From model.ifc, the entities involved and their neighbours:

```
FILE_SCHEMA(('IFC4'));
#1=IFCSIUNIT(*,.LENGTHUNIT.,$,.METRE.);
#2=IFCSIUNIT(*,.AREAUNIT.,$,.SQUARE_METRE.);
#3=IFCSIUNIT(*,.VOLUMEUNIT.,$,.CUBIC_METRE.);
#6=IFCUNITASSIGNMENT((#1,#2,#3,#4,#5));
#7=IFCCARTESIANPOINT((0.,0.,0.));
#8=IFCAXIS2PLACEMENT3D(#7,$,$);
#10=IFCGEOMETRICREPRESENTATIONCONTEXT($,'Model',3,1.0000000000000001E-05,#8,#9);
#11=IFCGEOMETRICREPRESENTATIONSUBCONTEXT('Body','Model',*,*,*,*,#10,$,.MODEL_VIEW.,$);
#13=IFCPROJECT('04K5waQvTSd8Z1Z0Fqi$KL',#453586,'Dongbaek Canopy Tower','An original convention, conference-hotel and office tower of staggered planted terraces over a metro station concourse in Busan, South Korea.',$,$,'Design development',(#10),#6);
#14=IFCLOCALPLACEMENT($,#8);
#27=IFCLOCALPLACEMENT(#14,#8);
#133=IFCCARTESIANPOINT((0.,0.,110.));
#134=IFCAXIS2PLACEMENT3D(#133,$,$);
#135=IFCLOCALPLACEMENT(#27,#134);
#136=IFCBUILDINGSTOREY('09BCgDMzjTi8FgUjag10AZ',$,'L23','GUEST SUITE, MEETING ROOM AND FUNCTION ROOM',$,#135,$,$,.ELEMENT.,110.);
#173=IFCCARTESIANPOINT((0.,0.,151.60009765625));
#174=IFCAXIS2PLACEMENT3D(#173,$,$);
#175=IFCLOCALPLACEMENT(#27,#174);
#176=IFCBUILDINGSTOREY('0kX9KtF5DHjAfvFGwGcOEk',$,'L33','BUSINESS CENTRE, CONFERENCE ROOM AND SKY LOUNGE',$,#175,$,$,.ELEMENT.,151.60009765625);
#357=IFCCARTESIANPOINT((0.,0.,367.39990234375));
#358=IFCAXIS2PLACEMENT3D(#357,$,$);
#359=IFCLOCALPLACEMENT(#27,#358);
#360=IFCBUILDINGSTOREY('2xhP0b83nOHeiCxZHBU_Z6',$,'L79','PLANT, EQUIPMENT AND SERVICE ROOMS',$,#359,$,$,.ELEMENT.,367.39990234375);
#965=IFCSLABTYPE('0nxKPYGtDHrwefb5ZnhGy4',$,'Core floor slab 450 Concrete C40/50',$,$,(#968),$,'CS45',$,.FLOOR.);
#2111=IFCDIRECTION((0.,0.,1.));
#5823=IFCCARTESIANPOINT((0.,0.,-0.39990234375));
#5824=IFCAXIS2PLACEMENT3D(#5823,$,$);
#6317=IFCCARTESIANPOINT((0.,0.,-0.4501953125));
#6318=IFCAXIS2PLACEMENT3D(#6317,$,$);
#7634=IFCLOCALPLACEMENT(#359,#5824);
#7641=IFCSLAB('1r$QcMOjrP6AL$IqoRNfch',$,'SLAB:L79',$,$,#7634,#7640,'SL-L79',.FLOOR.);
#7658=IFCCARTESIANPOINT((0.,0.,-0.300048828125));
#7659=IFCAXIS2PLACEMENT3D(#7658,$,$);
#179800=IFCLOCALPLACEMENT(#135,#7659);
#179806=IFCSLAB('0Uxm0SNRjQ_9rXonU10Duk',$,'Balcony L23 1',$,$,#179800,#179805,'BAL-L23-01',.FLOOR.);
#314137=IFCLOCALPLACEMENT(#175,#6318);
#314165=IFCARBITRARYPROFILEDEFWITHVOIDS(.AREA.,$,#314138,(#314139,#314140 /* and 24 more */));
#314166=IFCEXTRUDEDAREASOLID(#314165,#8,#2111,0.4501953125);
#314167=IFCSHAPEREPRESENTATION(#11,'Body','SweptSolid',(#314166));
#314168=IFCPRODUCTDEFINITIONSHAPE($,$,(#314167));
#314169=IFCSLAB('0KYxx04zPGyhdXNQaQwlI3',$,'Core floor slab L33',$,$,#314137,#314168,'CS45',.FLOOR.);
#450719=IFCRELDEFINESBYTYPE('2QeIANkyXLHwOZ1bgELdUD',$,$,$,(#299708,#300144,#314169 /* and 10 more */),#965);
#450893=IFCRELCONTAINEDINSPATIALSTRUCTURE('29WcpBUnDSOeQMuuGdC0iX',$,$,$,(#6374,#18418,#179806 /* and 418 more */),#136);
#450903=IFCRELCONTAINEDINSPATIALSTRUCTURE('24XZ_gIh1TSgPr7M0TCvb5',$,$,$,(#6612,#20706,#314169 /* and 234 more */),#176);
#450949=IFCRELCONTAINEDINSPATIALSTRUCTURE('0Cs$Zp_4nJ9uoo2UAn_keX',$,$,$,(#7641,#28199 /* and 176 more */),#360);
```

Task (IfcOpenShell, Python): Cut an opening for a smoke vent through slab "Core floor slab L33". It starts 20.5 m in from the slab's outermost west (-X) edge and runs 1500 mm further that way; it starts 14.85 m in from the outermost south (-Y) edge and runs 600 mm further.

```python
import numpy as np
import ifcopenshell
import ifcopenshell.api.feature
import ifcopenshell.api.geometry
import ifcopenshell.api.root
import ifcopenshell.geom
import ifcopenshell.util.placement
import ifcopenshell.util.representation
import ifcopenshell.util.shape
import ifcopenshell.util.unit

model = ifcopenshell.open("model.ifc")
unit_scale = ifcopenshell.util.unit.calculate_unit_scale(model)
settings = ifcopenshell.geom.settings()


def volume(element):
    """Net volume in cubic metres, openings subtracted."""
    shape = ifcopenshell.geom.create_shape(settings, element)
    return ifcopenshell.util.shape.get_volume(shape.geometry)


slab = model.by_id(314169)
before = volume(slab)

# Extent in the slab's own axes, in metres. The edges named are its -X and -Y sides.
slab_shape = ifcopenshell.geom.create_shape(settings, slab)
vertices = ifcopenshell.util.shape.get_vertices(slab_shape.geometry)
x_min, y_min, bottom = vertices.min(axis=0)
top = vertices[:, 2].max()

opening = ifcopenshell.api.root.create_entity(model, ifc_class="IfcOpeningElement", name="Smoke vent opening", predefined_type="OPENING")
context = ifcopenshell.util.representation.get_context(model, "Model", "Body", "MODEL_VIEW")
width, depth = 1.5, 0.6
outline = [(0.0, 0.0), (width, 0.0), (width, depth), (0.0, depth), (0.0, 0.0)]
# Overshoot both faces by 50 mm so the cut is clean.
shape = ifcopenshell.api.geometry.add_slab_representation(
    model, context=context, depth=top - bottom + 0.1, polyline=outline
)
ifcopenshell.api.geometry.assign_representation(model, product=opening, representation=shape)

matrix = ifcopenshell.util.placement.get_local_placement(slab.ObjectPlacement)
matrix[:, 3] = matrix @ np.append(np.array([x_min + 20.5, y_min + 14.85, bottom - 0.05]) / unit_scale, 1.0)
ifcopenshell.api.geometry.edit_object_placement(model, product=opening, matrix=matrix, is_si=False)
ifcopenshell.api.feature.add_feature(model, feature=opening, element=slab)

after = volume(slab)

print(f"slab volume {before:.3f} -> {after:.3f} m3")

model.write("model_edited.ifc")
```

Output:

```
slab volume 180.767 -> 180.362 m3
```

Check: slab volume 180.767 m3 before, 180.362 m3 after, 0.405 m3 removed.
